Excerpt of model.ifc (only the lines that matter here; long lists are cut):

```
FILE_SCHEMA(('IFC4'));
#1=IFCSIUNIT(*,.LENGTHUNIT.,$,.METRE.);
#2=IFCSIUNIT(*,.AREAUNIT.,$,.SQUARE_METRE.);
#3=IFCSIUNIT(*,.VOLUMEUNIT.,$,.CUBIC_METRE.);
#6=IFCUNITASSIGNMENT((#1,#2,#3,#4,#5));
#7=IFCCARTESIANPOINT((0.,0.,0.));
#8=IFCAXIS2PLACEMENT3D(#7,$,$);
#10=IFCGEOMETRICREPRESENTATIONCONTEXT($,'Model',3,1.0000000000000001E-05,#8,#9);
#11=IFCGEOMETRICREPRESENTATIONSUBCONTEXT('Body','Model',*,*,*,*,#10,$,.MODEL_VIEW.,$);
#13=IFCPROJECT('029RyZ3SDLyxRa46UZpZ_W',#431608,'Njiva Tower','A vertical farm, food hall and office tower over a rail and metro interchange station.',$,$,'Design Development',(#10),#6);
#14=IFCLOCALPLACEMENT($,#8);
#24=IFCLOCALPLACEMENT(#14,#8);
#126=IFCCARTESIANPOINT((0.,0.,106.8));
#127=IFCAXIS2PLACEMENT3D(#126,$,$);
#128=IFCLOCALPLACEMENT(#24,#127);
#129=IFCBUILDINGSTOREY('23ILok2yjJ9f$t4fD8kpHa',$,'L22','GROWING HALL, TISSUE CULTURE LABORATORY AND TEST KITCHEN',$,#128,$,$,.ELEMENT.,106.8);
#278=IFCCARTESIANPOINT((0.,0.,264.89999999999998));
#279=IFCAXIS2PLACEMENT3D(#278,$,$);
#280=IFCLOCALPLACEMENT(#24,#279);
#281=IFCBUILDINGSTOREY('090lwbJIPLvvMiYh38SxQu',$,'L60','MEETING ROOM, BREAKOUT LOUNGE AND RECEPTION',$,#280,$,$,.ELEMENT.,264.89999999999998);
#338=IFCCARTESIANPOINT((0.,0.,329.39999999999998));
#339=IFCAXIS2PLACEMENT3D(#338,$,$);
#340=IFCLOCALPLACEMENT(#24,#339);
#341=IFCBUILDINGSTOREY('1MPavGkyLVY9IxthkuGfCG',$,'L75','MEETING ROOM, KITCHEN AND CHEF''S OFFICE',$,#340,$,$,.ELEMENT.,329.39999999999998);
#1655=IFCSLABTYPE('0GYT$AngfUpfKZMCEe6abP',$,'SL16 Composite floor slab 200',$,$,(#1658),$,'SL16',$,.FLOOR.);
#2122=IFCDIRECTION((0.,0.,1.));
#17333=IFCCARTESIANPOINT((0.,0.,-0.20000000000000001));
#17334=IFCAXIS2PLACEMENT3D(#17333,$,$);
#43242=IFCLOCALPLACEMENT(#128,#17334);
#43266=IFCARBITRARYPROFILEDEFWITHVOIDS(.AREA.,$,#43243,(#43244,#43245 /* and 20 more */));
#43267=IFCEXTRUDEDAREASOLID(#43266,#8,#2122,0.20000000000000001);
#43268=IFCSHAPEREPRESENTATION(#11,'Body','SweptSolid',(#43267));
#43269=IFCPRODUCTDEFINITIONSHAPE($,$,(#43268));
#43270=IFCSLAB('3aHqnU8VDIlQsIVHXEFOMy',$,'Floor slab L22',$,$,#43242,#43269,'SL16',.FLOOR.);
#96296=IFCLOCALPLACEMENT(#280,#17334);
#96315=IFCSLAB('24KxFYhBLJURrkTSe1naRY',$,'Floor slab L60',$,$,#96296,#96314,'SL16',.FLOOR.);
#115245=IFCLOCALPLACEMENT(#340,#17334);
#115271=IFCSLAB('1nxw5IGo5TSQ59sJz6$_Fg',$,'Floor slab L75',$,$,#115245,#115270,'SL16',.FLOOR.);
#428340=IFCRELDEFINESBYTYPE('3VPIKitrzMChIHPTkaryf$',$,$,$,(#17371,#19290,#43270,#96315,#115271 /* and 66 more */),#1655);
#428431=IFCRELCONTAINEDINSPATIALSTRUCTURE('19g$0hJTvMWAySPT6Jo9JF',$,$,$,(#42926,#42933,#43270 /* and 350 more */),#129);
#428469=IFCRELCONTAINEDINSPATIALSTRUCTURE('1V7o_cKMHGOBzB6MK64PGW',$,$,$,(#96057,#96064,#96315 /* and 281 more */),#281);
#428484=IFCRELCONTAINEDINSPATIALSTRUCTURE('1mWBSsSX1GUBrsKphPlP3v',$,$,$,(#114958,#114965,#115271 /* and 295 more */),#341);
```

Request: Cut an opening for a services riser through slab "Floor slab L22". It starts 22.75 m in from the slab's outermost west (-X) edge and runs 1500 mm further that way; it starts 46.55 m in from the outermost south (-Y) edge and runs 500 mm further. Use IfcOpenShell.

```python
import numpy as np
import ifcopenshell
import ifcopenshell.api.feature
import ifcopenshell.api.geometry
import ifcopenshell.api.root
import ifcopenshell.geom
import ifcopenshell.util.placement
import ifcopenshell.util.representation
import ifcopenshell.util.shape
import ifcopenshell.util.unit

model = ifcopenshell.open("model.ifc")
unit_scale = ifcopenshell.util.unit.calculate_unit_scale(model)
settings = ifcopenshell.geom.settings()


def volume(element):
    """Net volume in cubic metres, openings subtracted."""
    shape = ifcopenshell.geom.create_shape(settings, element)
    return ifcopenshell.util.shape.get_volume(shape.geometry)


slab = model.by_guid("3aHqnU8VDIlQsIVHXEFOMy")
before = volume(slab)

# Extent in the slab's own axes, in metres. The edges named are its -X and -Y sides.
slab_shape = ifcopenshell.geom.create_shape(settings, slab)
vertices = ifcopenshell.util.shape.get_vertices(slab_shape.geometry)
x_min, y_min, bottom = vertices.min(axis=0)
top = vertices[:, 2].max()

opening = ifcopenshell.api.root.create_entity(model, ifc_class="IfcOpeningElement", name="Services riser opening", predefined_type="OPENING")
context = ifcopenshell.util.representation.get_context(model, "Model", "Body", "MODEL_VIEW")
width, depth = 1.5, 0.5
outline = [(0.0, 0.0), (width, 0.0), (width, depth), (0.0, depth), (0.0, 0.0)]
# Overshoot both faces by 50 mm so the cut is clean.
shape = ifcopenshell.api.geometry.add_slab_representation(
    model, context=context, depth=top - bottom + 0.1, polyline=outline
)
ifcopenshell.api.geometry.assign_representation(model, product=opening, representation=shape)

matrix = ifcopenshell.util.placement.get_local_placement(slab.ObjectPlacement)
matrix[:, 3] = matrix @ np.append(np.array([x_min + 22.75, y_min + 46.55, bottom - 0.05]) / unit_scale, 1.0)
ifcopenshell.api.geometry.edit_object_placement(model, product=opening, matrix=matrix, is_si=False)
ifcopenshell.api.feature.add_feature(model, feature=opening, element=slab)

after = volume(slab)

print(f"slab volume {before:.3f} -> {after:.3f} m3")

model.write("model-out.ifc")
```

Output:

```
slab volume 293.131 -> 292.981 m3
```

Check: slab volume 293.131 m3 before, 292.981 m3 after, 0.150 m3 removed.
